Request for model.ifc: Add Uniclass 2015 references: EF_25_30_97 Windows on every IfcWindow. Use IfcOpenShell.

First a look at what the model holds.

```python
import ifcopenshell

model = ifcopenshell.open("model.ifc")
print(model.schema)
print("classifications:", [c.Name for c in model.by_type("IfcClassification")])
for ifc_class in ("IfcDoor", "IfcRoof", "IfcStair", "IfcWall", "IfcWindow"):
    print(ifc_class, len(model.by_type(ifc_class)))
```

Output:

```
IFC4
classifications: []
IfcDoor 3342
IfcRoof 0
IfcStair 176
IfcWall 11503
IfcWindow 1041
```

```python
import ifcopenshell
import ifcopenshell.api.classification

model = ifcopenshell.open("model.ifc")

system = ifcopenshell.api.classification.add_classification(model, classification="Uniclass 2015")

codes = {
    "IfcWindow": ("EF_25_30_97", "Windows"),
}
for ifc_class, (code, name) in codes.items():
    products = model.by_type(ifc_class)
    ifcopenshell.api.classification.add_reference(
        model, products=products, classification=system, identification=code, name=name
    )
    print(code, len(products))

model.write("model_edited.ifc")
```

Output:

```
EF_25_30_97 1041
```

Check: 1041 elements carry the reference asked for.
